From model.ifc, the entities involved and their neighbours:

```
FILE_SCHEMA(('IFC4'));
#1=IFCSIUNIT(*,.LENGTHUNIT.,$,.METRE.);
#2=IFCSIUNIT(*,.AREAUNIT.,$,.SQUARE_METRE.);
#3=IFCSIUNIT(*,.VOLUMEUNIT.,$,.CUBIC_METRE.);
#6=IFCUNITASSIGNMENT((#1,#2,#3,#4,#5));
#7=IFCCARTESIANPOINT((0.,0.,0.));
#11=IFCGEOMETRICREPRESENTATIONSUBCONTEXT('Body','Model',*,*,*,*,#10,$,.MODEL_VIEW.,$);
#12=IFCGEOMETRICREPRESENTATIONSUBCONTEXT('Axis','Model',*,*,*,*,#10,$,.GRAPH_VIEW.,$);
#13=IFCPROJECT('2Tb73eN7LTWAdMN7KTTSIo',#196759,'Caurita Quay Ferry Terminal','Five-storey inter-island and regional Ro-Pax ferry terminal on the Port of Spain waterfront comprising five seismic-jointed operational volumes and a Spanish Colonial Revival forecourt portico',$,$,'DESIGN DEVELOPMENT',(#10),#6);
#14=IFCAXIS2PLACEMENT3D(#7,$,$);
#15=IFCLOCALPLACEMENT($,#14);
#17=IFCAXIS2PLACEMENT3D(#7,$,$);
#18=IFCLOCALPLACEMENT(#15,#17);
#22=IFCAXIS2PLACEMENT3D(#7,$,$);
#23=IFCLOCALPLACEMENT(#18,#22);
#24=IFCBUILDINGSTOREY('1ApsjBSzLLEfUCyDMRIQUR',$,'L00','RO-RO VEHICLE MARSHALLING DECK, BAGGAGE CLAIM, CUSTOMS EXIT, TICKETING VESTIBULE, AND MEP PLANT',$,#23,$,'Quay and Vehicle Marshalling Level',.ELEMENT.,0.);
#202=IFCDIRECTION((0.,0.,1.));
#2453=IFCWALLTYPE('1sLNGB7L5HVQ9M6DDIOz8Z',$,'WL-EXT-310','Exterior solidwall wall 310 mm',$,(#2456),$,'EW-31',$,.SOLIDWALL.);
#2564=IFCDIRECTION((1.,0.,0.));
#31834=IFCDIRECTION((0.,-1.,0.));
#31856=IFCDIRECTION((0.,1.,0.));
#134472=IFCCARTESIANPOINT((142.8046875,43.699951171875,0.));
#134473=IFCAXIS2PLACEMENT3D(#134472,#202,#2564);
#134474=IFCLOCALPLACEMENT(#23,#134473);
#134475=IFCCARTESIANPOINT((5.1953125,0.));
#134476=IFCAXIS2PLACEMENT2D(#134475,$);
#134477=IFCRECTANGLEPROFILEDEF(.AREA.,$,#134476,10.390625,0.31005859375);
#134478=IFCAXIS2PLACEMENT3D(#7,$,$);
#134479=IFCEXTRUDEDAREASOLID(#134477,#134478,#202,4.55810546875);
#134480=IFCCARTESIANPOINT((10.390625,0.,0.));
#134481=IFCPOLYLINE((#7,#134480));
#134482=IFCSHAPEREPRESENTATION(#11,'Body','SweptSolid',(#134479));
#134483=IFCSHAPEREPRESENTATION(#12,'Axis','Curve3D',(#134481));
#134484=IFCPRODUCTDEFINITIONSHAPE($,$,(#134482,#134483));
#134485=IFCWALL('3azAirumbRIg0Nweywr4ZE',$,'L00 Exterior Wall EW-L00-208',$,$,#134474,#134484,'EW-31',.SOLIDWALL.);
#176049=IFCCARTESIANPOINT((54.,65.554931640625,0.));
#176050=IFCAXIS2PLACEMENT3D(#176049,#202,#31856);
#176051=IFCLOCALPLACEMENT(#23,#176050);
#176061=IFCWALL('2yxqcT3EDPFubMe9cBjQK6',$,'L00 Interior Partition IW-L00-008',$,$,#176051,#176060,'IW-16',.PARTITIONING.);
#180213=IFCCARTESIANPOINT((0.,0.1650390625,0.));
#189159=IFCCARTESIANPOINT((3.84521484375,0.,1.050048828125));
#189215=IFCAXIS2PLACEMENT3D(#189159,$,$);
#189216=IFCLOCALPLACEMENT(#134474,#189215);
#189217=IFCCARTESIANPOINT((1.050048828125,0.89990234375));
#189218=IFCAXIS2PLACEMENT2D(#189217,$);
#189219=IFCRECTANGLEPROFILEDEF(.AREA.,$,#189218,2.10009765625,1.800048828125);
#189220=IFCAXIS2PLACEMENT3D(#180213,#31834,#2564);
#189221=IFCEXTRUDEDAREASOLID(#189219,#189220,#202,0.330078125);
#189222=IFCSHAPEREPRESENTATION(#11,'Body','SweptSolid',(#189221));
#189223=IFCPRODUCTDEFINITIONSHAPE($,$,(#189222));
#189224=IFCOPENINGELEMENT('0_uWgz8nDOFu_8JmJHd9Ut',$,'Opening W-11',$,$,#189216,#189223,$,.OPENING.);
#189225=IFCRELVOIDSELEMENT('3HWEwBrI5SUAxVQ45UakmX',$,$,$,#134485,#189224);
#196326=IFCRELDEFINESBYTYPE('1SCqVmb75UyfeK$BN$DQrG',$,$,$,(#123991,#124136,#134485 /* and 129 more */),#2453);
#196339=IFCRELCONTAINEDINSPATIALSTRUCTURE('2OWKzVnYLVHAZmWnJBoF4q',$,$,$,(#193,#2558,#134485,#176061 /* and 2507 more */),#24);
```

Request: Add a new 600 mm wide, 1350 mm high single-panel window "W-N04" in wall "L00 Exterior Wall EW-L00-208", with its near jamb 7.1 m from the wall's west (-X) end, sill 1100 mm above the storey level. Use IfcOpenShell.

```python
import numpy as np
import ifcopenshell
import ifcopenshell.api.feature
import ifcopenshell.api.geometry
import ifcopenshell.api.root
import ifcopenshell.api.spatial
import ifcopenshell.geom
import ifcopenshell.util.element
import ifcopenshell.util.placement
import ifcopenshell.util.representation
import ifcopenshell.util.shape
import ifcopenshell.util.unit

model = ifcopenshell.open("model.ifc")
unit_scale = ifcopenshell.util.unit.calculate_unit_scale(model)
settings = ifcopenshell.geom.settings()


def volume(element):
    """Net volume in cubic metres, openings subtracted."""
    shape = ifcopenshell.geom.create_shape(settings, element)
    return ifcopenshell.util.shape.get_volume(shape.geometry)


wall = model.by_guid("3azAirumbRIg0Nweywr4ZE")
storey = ifcopenshell.util.element.get_container(wall, ifc_class="IfcBuildingStorey")
context = ifcopenshell.util.representation.get_context(model, "Model", "Body", "MODEL_VIEW")
before = volume(wall)

width, height, from_end, sill = 0.6, 1.35, 7.1, 1.1  # metres

# The wall runs along its own X axis, and the end named is its -X end.
wall_shape = ifcopenshell.geom.create_shape(settings, wall)
x, y, z = ifcopenshell.util.shape.get_vertices(wall_shape.geometry).T
start = x.min() + from_end
face, thickness = float(y.min()), float(y.max() - y.min())
wall_matrix = ifcopenshell.util.placement.get_local_placement(wall.ObjectPlacement)
level = ifcopenshell.util.placement.get_local_placement(storey.ObjectPlacement)[2, 3]


def in_wall(x, y):
    """Placement at x, y metres in the wall's axes, at sill height."""
    matrix = wall_matrix.copy()
    matrix[:, 3] = wall_matrix @ np.array([x / unit_scale, y / unit_scale, 0.0, 1.0])
    matrix[2, 3] = level + sill / unit_scale
    return matrix


# Opening: a box that overshoots both wall faces by 50 mm.
opening = ifcopenshell.api.root.create_entity(model, ifc_class="IfcOpeningElement", predefined_type="OPENING")
box = ifcopenshell.api.geometry.add_wall_representation(
    model, context=context, length=width, height=height, thickness=thickness + 0.1
)
ifcopenshell.api.geometry.assign_representation(model, product=opening, representation=box)
ifcopenshell.api.geometry.edit_object_placement(model, product=opening, matrix=in_wall(start, face - 0.05), is_si=False)
ifcopenshell.api.feature.add_feature(model, feature=opening, element=wall)

window = ifcopenshell.api.root.create_entity(model, ifc_class="IfcWindow", name="W-N04", predefined_type="WINDOW")
window.OverallWidth, window.OverallHeight = width / unit_scale, height / unit_scale
window.PartitioningType = "SINGLE_PANEL"
body = ifcopenshell.api.geometry.add_window_representation(
    model,
    context=context,
    overall_width=window.OverallWidth,
    overall_height=window.OverallHeight,
    partition_type="SINGLE_PANEL",
)
ifcopenshell.api.geometry.assign_representation(model, product=window, representation=body)
ifcopenshell.api.spatial.assign_container(model, products=[window], relating_structure=storey)
ifcopenshell.api.feature.add_filling(model, opening=opening, element=window)

# Centre the window in the wall's thickness.
ifcopenshell.api.geometry.edit_object_placement(model, product=window, matrix=in_wall(start, face), is_si=False)
window_shape = ifcopenshell.geom.create_shape(settings, window)
depth = ifcopenshell.util.shape.get_vertices(window_shape.geometry)[:, 1]
offset = face + thickness / 2 - (depth.min() + depth.max()) / 2
ifcopenshell.api.geometry.edit_object_placement(model, product=window, matrix=in_wall(start, offset), is_si=False)

after = volume(wall)

print(f"wall volume {before:.3f} -> {after:.3f} m3")

model.write("model_rev.ifc")
```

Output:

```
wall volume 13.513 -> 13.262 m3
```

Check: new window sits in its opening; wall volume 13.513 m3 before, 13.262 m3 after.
